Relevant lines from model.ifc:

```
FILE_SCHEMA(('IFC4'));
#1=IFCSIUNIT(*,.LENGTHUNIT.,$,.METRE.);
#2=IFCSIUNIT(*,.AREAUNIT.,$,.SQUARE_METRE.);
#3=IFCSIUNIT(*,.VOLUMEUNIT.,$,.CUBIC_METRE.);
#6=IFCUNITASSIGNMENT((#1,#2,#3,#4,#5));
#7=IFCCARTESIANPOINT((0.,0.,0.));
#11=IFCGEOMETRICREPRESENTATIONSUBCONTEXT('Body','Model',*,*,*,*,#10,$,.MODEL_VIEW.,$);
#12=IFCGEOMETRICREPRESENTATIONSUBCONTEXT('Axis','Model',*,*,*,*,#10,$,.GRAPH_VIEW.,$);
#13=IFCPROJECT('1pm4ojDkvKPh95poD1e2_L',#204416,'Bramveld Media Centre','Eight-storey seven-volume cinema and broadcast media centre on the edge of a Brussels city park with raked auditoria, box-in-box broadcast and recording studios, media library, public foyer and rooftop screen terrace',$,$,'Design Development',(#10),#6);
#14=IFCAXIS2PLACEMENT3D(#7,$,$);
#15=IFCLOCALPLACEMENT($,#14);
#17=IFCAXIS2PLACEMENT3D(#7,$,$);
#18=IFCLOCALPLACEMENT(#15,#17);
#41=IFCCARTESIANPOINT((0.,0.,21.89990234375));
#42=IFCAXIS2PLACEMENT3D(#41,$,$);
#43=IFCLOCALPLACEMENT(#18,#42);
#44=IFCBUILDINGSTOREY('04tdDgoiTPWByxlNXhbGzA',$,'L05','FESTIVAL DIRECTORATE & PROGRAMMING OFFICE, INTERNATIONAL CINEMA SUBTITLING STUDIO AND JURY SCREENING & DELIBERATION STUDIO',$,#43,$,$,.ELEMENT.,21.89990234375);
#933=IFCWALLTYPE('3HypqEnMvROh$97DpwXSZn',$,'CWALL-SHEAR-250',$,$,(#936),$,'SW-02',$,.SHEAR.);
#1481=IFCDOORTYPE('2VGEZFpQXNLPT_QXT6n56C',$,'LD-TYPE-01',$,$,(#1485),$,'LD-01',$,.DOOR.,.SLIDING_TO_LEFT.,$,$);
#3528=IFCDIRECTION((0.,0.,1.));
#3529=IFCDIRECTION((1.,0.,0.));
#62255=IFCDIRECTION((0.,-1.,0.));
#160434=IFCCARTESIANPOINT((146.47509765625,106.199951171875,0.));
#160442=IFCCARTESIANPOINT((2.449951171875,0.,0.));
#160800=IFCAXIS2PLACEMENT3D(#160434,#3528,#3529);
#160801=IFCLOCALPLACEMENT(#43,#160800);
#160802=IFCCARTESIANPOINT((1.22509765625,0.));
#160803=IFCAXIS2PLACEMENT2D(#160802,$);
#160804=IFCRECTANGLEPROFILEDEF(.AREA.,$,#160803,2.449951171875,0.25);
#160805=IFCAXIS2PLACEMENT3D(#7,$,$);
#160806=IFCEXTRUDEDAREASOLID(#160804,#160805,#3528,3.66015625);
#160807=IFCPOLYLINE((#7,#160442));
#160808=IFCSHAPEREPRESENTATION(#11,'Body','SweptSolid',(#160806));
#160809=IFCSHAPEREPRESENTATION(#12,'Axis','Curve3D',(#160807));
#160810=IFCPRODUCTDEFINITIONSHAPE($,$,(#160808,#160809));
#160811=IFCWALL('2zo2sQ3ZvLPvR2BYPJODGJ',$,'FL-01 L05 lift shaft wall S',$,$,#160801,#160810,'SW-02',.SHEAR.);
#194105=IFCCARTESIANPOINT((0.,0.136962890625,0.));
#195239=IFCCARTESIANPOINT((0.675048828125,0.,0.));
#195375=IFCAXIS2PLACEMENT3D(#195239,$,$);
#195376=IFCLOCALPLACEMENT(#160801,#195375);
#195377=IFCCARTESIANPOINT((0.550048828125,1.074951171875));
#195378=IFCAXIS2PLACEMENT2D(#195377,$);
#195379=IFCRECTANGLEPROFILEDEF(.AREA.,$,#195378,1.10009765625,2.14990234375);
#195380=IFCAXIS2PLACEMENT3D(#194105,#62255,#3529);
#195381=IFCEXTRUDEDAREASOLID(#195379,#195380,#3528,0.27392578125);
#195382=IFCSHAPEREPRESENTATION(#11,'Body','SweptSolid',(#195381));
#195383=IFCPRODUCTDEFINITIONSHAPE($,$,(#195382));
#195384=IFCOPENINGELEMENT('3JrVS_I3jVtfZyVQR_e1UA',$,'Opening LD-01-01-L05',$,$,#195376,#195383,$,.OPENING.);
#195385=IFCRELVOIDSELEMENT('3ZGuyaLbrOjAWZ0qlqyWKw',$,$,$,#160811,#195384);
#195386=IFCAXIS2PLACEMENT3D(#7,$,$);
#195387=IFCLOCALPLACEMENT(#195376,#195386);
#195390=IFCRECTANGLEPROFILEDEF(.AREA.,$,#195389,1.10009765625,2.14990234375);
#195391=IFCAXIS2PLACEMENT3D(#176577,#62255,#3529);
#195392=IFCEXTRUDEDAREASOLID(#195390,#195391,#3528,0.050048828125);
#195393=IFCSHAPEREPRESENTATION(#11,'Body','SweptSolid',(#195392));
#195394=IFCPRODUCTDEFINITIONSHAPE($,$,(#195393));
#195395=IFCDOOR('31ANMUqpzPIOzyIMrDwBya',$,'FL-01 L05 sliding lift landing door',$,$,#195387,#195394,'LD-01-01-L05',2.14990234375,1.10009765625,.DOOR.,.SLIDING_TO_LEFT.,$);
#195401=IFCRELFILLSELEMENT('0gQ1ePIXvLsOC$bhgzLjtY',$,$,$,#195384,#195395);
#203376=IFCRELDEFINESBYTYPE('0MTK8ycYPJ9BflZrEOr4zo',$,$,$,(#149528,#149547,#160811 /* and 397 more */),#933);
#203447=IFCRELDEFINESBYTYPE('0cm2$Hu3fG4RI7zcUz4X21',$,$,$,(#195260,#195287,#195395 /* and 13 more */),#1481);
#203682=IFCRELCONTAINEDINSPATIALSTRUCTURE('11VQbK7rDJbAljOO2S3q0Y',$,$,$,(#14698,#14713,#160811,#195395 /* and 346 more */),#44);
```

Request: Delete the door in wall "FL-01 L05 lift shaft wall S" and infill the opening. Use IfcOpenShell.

```python
import ifcopenshell
import ifcopenshell.api.feature
import ifcopenshell.api.root
import ifcopenshell.geom
import ifcopenshell.util.shape

model = ifcopenshell.open("model.ifc")
settings = ifcopenshell.geom.settings()


def volume(element):
    """Net volume in cubic metres, openings subtracted."""
    shape = ifcopenshell.geom.create_shape(settings, element)
    return ifcopenshell.util.shape.get_volume(shape.geometry)


door = model.by_guid("31ANMUqpzPIOzyIMrDwBya")
opening = door.FillsVoids[0].RelatingOpeningElement
wall = opening.VoidsElements[0].RelatingBuildingElement
before = volume(wall)

ifcopenshell.api.root.remove_product(model, product=door)
ifcopenshell.api.feature.remove_feature(model, feature=opening)

after = volume(wall)

print(f"wall volume {before:.3f} -> {after:.3f} m3")

model.write("model_updated.ifc")
```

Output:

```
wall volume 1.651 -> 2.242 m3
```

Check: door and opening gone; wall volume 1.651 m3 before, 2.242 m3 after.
